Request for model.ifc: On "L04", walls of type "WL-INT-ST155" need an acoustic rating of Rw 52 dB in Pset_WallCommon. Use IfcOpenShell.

First a look at what the model holds.

```python
import ifcopenshell
import ifcopenshell.util.element

model = ifcopenshell.open("model.ifc")
print(model.schema)
storey = next(s for s in model.by_type("IfcBuildingStorey") if s.Name == "L04")
walls = [e for e in ifcopenshell.util.element.get_decomposition(storey) if e.is_a("IfcWall")]
seen = {}
for e in walls:
    element_type = ifcopenshell.util.element.get_type(e)
    key = (element_type.Name if element_type != e and element_type else None, ifcopenshell.util.element.get_pset(e, "Pset_WallCommon", "AcousticRating"))
    seen[key] = seen.get(key, 0) + 1
for (name, value), count in sorted(seen.items(), key=str):
    print(count, "x", name, "|", value)
```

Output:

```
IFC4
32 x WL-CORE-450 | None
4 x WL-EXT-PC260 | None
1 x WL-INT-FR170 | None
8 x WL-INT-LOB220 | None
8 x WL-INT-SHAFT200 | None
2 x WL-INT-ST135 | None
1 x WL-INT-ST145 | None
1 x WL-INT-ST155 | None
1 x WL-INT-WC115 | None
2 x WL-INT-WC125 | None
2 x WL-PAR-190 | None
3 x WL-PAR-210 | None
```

```python
import ifcopenshell
import ifcopenshell.api.pset
import ifcopenshell.util.element

model = ifcopenshell.open("model.ifc")

storey = next(s for s in model.by_type("IfcBuildingStorey") if s.Name == "L04")
walls = [e for e in ifcopenshell.util.element.get_decomposition(storey) if e.is_a("IfcWall")]

count = 0
for e in walls:
    element_type = ifcopenshell.util.element.get_type(e)
    if element_type in (None, e) or element_type.Name != "WL-INT-ST155":
        continue
    # add_pset returns the element's existing set when there is one.
    pset = ifcopenshell.api.pset.add_pset(model, product=e, name="Pset_WallCommon")
    ifcopenshell.api.pset.edit_pset(model, pset=pset, properties={"AcousticRating": "Rw 52 dB"})
    count += 1

print(count, "walls updated")

model.write("model_rev.ifc")
```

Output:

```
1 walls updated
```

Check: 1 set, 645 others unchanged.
